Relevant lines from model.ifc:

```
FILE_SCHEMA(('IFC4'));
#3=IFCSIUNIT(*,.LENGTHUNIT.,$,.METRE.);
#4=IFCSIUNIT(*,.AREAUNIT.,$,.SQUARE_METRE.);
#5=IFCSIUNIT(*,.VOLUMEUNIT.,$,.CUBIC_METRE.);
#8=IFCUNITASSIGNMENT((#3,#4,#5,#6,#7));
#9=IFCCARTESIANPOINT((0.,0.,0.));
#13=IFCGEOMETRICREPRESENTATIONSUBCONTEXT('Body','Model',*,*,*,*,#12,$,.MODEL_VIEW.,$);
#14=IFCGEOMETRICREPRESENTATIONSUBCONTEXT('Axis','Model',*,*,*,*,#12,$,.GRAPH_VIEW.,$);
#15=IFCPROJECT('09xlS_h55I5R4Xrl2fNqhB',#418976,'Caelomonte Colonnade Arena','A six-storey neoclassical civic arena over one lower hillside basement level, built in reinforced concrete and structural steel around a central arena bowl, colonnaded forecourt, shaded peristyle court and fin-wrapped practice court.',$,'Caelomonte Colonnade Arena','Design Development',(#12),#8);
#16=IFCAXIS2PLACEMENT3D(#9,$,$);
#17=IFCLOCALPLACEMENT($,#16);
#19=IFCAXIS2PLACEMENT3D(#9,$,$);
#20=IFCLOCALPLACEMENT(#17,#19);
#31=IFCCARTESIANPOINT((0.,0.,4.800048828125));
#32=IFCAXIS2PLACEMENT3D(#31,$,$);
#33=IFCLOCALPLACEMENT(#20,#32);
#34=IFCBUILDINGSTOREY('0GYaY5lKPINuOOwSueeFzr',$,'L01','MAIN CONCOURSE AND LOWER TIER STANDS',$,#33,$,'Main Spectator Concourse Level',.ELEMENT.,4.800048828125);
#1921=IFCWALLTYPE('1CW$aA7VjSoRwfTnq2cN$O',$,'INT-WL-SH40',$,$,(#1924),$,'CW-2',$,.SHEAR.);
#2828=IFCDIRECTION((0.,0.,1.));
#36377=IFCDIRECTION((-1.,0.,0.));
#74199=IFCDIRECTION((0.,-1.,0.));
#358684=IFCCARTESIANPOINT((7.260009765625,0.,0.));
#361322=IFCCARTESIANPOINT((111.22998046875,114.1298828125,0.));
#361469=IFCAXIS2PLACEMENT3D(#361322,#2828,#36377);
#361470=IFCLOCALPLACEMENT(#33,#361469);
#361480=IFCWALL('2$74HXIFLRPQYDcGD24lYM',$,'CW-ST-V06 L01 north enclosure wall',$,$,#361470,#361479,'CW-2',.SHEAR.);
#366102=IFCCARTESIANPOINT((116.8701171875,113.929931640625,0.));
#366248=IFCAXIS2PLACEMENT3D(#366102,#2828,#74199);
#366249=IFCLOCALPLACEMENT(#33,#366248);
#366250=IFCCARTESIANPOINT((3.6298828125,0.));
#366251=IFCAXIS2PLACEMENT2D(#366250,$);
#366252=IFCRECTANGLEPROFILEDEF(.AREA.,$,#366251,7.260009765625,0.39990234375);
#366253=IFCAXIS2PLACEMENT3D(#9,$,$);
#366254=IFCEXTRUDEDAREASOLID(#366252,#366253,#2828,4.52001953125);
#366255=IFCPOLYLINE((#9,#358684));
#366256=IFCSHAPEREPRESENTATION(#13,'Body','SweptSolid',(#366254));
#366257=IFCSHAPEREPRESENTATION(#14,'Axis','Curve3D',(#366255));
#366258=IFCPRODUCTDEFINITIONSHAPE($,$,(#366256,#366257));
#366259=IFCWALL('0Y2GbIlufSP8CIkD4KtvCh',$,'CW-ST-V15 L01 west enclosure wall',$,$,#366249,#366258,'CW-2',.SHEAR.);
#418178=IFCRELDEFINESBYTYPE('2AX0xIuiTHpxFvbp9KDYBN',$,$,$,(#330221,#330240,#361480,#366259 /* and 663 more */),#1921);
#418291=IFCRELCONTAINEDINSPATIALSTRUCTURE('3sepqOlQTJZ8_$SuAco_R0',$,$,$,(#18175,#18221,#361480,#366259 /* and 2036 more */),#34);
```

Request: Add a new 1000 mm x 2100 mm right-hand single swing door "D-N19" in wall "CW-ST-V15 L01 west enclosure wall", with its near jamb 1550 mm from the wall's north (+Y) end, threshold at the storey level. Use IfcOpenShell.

```python
import numpy as np
import ifcopenshell
import ifcopenshell.api.feature
import ifcopenshell.api.geometry
import ifcopenshell.api.root
import ifcopenshell.api.spatial
import ifcopenshell.geom
import ifcopenshell.util.element
import ifcopenshell.util.placement
import ifcopenshell.util.representation
import ifcopenshell.util.shape
import ifcopenshell.util.unit

model = ifcopenshell.open("model.ifc")
unit_scale = ifcopenshell.util.unit.calculate_unit_scale(model)
settings = ifcopenshell.geom.settings()


def volume(element):
    """Net volume in cubic metres, openings subtracted."""
    shape = ifcopenshell.geom.create_shape(settings, element)
    return ifcopenshell.util.shape.get_volume(shape.geometry)


wall = model.by_guid("0Y2GbIlufSP8CIkD4KtvCh")
storey = ifcopenshell.util.element.get_container(wall, ifc_class="IfcBuildingStorey")
context = ifcopenshell.util.representation.get_context(model, "Model", "Body", "MODEL_VIEW")
before = volume(wall)

width, height, from_end, sill = 1, 2.1, 1.55, 0.0  # metres

# The wall runs along its own X axis, and the end named is its -X end.
wall_shape = ifcopenshell.geom.create_shape(settings, wall)
x, y, z = ifcopenshell.util.shape.get_vertices(wall_shape.geometry).T
start = x.min() + from_end
face, thickness = float(y.min()), float(y.max() - y.min())
wall_matrix = ifcopenshell.util.placement.get_local_placement(wall.ObjectPlacement)
level = ifcopenshell.util.placement.get_local_placement(storey.ObjectPlacement)[2, 3]


def in_wall(x, y):
    """Placement at x, y metres in the wall's axes, at sill height."""
    matrix = wall_matrix.copy()
    matrix[:, 3] = wall_matrix @ np.array([x / unit_scale, y / unit_scale, 0.0, 1.0])
    matrix[2, 3] = level + sill / unit_scale
    return matrix


# Opening: a box that overshoots both wall faces by 50 mm.
opening = ifcopenshell.api.root.create_entity(model, ifc_class="IfcOpeningElement", predefined_type="OPENING")
box = ifcopenshell.api.geometry.add_wall_representation(
    model, context=context, length=width, height=height, thickness=thickness + 0.1
)
ifcopenshell.api.geometry.assign_representation(model, product=opening, representation=box)
ifcopenshell.api.geometry.edit_object_placement(model, product=opening, matrix=in_wall(start, face - 0.05), is_si=False)
ifcopenshell.api.feature.add_feature(model, feature=opening, element=wall)

door = ifcopenshell.api.root.create_entity(model, ifc_class="IfcDoor", name="D-N19", predefined_type="DOOR")
door.OverallWidth, door.OverallHeight = width / unit_scale, height / unit_scale
door.OperationType = "SINGLE_SWING_RIGHT"
body = ifcopenshell.api.geometry.add_door_representation(
    model,
    context=context,
    overall_width=door.OverallWidth,
    overall_height=door.OverallHeight,
    operation_type="SINGLE_SWING_RIGHT",
    lining_properties={"LiningDepth": thickness / unit_scale, "ThresholdDepth": thickness / unit_scale},
)
ifcopenshell.api.geometry.assign_representation(model, product=door, representation=body)
ifcopenshell.api.spatial.assign_container(model, products=[door], relating_structure=storey)
ifcopenshell.api.feature.add_filling(model, opening=opening, element=door)

# The lining spans the wall, so the door starts at the wall face.
ifcopenshell.api.geometry.edit_object_placement(model, product=door, matrix=in_wall(start, face), is_si=False)

after = volume(wall)

print(f"wall volume {before:.3f} -> {after:.3f} m3")

model.write("model-out.ifc")
```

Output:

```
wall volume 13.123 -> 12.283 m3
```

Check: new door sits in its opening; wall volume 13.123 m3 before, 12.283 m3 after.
